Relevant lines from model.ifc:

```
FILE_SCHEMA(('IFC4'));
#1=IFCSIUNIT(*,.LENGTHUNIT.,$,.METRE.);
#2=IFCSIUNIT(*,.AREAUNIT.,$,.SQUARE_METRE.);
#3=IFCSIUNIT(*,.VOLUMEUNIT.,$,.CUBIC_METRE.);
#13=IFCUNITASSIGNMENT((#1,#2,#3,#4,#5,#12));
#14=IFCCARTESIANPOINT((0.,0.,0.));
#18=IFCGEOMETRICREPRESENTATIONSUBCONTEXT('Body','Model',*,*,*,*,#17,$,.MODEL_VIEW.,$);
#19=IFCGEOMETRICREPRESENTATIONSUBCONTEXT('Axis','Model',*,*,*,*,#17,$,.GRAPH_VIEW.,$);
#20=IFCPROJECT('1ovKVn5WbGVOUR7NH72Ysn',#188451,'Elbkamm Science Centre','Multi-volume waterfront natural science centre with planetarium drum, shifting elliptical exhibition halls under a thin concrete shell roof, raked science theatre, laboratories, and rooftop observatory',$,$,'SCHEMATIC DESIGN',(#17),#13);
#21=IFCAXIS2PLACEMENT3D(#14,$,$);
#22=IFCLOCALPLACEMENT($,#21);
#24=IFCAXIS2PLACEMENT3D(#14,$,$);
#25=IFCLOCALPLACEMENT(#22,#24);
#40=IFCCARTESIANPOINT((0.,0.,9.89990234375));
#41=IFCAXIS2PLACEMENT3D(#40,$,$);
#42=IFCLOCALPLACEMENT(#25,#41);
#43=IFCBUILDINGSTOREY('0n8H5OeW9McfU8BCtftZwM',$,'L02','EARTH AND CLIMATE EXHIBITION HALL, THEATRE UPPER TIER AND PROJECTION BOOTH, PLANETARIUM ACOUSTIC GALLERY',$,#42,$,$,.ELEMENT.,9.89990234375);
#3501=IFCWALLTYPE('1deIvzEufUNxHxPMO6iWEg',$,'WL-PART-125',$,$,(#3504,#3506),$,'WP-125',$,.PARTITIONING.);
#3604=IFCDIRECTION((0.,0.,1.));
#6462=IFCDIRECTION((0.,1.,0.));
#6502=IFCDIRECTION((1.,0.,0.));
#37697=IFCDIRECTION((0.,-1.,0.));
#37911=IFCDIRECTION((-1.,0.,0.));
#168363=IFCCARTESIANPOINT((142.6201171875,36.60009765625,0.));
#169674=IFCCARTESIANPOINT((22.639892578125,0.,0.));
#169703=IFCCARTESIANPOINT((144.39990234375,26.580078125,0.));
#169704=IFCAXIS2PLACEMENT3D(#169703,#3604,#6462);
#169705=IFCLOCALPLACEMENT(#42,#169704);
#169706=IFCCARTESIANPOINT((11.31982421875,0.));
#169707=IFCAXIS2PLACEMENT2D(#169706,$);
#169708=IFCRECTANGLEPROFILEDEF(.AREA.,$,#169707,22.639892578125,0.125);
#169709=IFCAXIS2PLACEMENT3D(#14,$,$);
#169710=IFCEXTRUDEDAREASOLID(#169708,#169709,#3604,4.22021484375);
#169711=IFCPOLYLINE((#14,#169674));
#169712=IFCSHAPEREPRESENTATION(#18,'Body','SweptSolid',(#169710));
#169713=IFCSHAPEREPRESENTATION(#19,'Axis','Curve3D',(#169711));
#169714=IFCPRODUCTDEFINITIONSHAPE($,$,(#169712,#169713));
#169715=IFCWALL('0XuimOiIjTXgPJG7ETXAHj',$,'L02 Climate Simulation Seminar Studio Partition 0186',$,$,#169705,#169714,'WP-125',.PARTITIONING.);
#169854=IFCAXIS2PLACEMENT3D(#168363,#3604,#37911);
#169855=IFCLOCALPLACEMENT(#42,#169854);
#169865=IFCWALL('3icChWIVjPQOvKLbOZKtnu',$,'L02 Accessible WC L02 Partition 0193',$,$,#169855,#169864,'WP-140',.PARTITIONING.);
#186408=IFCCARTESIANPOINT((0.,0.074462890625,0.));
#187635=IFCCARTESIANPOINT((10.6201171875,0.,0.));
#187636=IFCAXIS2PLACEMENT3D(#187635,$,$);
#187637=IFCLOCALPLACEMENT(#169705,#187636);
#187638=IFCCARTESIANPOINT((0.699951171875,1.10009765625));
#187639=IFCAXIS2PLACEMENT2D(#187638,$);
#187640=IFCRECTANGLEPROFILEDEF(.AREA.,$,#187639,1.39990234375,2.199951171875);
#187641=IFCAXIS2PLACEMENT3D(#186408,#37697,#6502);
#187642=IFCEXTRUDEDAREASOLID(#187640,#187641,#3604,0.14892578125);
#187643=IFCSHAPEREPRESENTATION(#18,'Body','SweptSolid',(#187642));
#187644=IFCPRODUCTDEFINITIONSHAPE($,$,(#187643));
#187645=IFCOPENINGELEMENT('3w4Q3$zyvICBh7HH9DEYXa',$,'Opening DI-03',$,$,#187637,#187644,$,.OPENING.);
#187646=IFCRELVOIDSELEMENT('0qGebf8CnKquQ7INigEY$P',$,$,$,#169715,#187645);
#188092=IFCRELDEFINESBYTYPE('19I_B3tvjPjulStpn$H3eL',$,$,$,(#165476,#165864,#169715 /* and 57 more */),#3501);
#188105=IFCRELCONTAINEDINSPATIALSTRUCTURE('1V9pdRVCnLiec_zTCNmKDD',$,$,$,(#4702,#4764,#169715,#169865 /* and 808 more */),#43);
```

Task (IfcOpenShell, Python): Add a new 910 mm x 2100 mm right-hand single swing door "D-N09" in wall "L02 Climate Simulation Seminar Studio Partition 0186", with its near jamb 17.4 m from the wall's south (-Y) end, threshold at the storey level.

```python
import numpy as np
import ifcopenshell
import ifcopenshell.api.feature
import ifcopenshell.api.geometry
import ifcopenshell.api.root
import ifcopenshell.api.spatial
import ifcopenshell.geom
import ifcopenshell.util.element
import ifcopenshell.util.placement
import ifcopenshell.util.representation
import ifcopenshell.util.shape
import ifcopenshell.util.unit

model = ifcopenshell.open("model.ifc")
unit_scale = ifcopenshell.util.unit.calculate_unit_scale(model)
settings = ifcopenshell.geom.settings()


def volume(element):
    """Net volume in cubic metres, openings subtracted."""
    shape = ifcopenshell.geom.create_shape(settings, element)
    return ifcopenshell.util.shape.get_volume(shape.geometry)


wall = model.by_id(169715)
storey = ifcopenshell.util.element.get_container(wall, ifc_class="IfcBuildingStorey")
context = ifcopenshell.util.representation.get_context(model, "Model", "Body", "MODEL_VIEW")
before = volume(wall)

width, height, from_end, sill = 0.91, 2.1, 17.4, 0.0  # metres

# The wall runs along its own X axis, and the end named is its -X end.
wall_shape = ifcopenshell.geom.create_shape(settings, wall)
x, y, z = ifcopenshell.util.shape.get_vertices(wall_shape.geometry).T
start = x.min() + from_end
face, thickness = float(y.min()), float(y.max() - y.min())
wall_matrix = ifcopenshell.util.placement.get_local_placement(wall.ObjectPlacement)
level = ifcopenshell.util.placement.get_local_placement(storey.ObjectPlacement)[2, 3]


def in_wall(x, y):
    """Placement at x, y metres in the wall's axes, at sill height."""
    matrix = wall_matrix.copy()
    matrix[:, 3] = wall_matrix @ np.array([x / unit_scale, y / unit_scale, 0.0, 1.0])
    matrix[2, 3] = level + sill / unit_scale
    return matrix


# Opening: a box that overshoots both wall faces by 50 mm.
opening = ifcopenshell.api.root.create_entity(model, ifc_class="IfcOpeningElement", predefined_type="OPENING")
box = ifcopenshell.api.geometry.add_wall_representation(
    model, context=context, length=width, height=height, thickness=thickness + 0.1
)
ifcopenshell.api.geometry.assign_representation(model, product=opening, representation=box)
ifcopenshell.api.geometry.edit_object_placement(model, product=opening, matrix=in_wall(start, face - 0.05), is_si=False)
ifcopenshell.api.feature.add_feature(model, feature=opening, element=wall)

door = ifcopenshell.api.root.create_entity(model, ifc_class="IfcDoor", name="D-N09", predefined_type="DOOR")
door.OverallWidth, door.OverallHeight = width / unit_scale, height / unit_scale
door.OperationType = "SINGLE_SWING_RIGHT"
body = ifcopenshell.api.geometry.add_door_representation(
    model,
    context=context,
    overall_width=door.OverallWidth,
    overall_height=door.OverallHeight,
    operation_type="SINGLE_SWING_RIGHT",
    lining_properties={"LiningDepth": thickness / unit_scale, "ThresholdDepth": thickness / unit_scale},
)
ifcopenshell.api.geometry.assign_representation(model, product=door, representation=body)
ifcopenshell.api.spatial.assign_container(model, products=[door], relating_structure=storey)
ifcopenshell.api.feature.add_filling(model, opening=opening, element=door)

# The lining spans the wall, so the door starts at the wall face.
ifcopenshell.api.geometry.edit_object_placement(model, product=door, matrix=in_wall(start, face), is_si=False)

after = volume(wall)

print(f"wall volume {before:.3f} -> {after:.3f} m3")

model.write("model_edited.ifc")
```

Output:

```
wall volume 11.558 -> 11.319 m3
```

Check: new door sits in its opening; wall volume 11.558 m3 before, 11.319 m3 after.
